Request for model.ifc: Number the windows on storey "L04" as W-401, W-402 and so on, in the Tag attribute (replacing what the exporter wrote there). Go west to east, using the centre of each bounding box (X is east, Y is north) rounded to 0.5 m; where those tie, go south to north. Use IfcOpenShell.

First a look at what the model holds.

```python
import ifcopenshell
import ifcopenshell.util.element
import ifcopenshell.util.placement

model = ifcopenshell.open("model.ifc")
print(model.schema)
storey = next(s for s in model.by_type("IfcBuildingStorey") if s.Name == "L04")
windows = [e for e in ifcopenshell.util.element.get_decomposition(storey) if e.is_a("IfcWindow")]
for e in sorted(windows, key=lambda e: e.id()):
    origin = ifcopenshell.util.placement.get_local_placement(e.ObjectPlacement)[:3, 3]
    print(e.id(), e.Tag, e.Name, origin.round(2) + 0.0, sep=" | ")
```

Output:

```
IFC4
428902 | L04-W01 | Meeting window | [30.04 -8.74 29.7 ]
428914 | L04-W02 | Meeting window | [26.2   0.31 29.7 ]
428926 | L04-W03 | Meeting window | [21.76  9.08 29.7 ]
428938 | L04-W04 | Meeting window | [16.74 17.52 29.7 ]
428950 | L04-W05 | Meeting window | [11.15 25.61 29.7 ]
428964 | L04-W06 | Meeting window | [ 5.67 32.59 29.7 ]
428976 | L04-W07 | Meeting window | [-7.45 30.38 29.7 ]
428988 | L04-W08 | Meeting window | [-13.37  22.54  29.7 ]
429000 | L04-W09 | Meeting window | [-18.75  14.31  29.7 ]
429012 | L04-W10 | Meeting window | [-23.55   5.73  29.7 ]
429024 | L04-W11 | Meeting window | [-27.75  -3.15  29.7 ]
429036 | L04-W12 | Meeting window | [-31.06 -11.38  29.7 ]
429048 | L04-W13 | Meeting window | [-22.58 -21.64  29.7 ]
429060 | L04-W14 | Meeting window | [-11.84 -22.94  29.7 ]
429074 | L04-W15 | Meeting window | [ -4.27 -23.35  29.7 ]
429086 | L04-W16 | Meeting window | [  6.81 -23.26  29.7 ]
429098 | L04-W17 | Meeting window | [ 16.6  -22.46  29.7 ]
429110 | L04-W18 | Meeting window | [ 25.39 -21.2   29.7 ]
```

```python
import ifcopenshell
import ifcopenshell.geom
import ifcopenshell.util.element
import ifcopenshell.util.shape

model = ifcopenshell.open("model.ifc")
settings = ifcopenshell.geom.settings()
settings.set("use-world-coords", True)


def centre(element):
    shape = ifcopenshell.geom.create_shape(settings, element)
    return ifcopenshell.util.shape.get_bbox_centroid(shape.geometry)


storey = next(s for s in model.by_type("IfcBuildingStorey") if s.Name == "L04")
windows = [e for e in ifcopenshell.util.element.get_decomposition(storey) if e.is_a("IfcWindow")]

# Insertion points can sit at a corner or the storey origin, so sort by the geometry (in metres).
centres = {e: centre(e) for e in windows}
windows.sort(key=lambda e: (round(centres[e][0] / 0.5), centres[e][1]))

for i, e in enumerate(windows, start=1):
    number = f"W-4{i:02d}"
    e.Tag = number
    print(e.id(), number)

model.write("model_v2.ifc")
```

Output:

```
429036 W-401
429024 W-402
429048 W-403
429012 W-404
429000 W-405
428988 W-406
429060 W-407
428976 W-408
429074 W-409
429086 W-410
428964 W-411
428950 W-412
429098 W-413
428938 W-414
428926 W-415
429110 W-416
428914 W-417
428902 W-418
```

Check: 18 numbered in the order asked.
